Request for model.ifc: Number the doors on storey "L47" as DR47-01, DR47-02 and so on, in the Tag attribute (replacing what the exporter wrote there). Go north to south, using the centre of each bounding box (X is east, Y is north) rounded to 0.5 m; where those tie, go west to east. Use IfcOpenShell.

First a look at what the model holds.

```python
import ifcopenshell
import ifcopenshell.util.element
import ifcopenshell.util.placement

model = ifcopenshell.open("model.ifc")
print(model.schema)
storey = next(s for s in model.by_type("IfcBuildingStorey") if s.Name == "L47")
doors = [e for e in ifcopenshell.util.element.get_decomposition(storey) if e.is_a("IfcDoor")]
for e in sorted(doors, key=lambda e: e.id()):
    origin = ifcopenshell.util.placement.get_local_placement(e.ObjectPlacement)[:3, 3]
    print(e.id(), e.Tag, e.Name, origin.round(2) + 0.0, sep=" | ")
```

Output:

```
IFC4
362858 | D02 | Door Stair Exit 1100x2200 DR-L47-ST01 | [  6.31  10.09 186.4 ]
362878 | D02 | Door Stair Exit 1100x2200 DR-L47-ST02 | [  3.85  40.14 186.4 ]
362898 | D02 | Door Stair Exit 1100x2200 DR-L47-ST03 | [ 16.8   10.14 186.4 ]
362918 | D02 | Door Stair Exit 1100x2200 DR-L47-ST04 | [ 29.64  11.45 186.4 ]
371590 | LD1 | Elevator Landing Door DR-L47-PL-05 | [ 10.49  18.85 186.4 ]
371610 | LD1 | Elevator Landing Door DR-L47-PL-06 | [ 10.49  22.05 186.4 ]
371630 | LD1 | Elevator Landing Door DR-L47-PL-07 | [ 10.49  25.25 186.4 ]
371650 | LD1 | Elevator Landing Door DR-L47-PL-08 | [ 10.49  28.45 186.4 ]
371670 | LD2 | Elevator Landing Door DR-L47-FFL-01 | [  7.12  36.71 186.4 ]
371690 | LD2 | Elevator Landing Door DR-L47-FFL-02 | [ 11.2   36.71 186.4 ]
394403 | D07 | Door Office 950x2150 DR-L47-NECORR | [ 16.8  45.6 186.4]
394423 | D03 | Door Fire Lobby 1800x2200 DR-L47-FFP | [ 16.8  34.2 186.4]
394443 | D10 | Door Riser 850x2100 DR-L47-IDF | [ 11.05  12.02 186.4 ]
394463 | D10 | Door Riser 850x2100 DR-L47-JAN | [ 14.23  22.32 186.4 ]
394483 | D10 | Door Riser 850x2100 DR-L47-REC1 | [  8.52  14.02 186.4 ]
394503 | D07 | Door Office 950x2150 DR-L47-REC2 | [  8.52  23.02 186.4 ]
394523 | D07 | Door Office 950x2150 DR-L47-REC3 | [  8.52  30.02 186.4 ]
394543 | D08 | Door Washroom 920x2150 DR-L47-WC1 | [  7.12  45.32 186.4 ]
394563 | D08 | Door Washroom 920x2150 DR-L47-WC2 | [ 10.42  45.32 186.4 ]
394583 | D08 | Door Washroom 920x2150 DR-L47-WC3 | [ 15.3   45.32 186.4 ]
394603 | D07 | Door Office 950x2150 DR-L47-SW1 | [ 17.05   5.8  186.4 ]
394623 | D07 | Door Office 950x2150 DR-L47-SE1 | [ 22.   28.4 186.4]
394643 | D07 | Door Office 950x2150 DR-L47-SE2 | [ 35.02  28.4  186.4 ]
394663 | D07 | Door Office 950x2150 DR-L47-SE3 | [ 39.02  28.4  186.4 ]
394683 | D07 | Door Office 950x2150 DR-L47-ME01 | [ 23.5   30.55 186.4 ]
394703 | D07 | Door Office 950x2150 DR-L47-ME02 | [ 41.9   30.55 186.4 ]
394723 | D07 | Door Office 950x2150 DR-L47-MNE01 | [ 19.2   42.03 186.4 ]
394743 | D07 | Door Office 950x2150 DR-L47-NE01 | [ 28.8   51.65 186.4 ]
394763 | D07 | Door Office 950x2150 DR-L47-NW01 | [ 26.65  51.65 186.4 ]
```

```python
import ifcopenshell
import ifcopenshell.geom
import ifcopenshell.util.element
import ifcopenshell.util.shape

model = ifcopenshell.open("model.ifc")
settings = ifcopenshell.geom.settings()
settings.set("use-world-coords", True)


def centre(element):
    shape = ifcopenshell.geom.create_shape(settings, element)
    return ifcopenshell.util.shape.get_bbox_centroid(shape.geometry)


storey = next(s for s in model.by_type("IfcBuildingStorey") if s.Name == "L47")
doors = [e for e in ifcopenshell.util.element.get_decomposition(storey) if e.is_a("IfcDoor")]

# Insertion points can sit at a corner or the storey origin, so sort by the geometry (in metres).
centres = {e: centre(e) for e in doors}
doors.sort(key=lambda e: (-round(centres[e][1] / 0.5), centres[e][0]))

for i, e in enumerate(doors, start=1):
    number = f"DR47-{i:02d}"
    e.Tag = number
    print(e.id(), number)

model.write("model_rev.ifc")
```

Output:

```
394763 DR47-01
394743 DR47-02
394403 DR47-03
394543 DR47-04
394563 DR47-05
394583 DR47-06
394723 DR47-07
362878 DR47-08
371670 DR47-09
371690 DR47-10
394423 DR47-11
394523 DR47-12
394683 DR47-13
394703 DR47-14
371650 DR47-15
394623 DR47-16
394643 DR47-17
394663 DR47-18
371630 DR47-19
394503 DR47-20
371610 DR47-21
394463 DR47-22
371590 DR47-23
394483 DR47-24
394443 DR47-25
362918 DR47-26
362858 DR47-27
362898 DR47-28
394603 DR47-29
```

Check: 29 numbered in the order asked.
